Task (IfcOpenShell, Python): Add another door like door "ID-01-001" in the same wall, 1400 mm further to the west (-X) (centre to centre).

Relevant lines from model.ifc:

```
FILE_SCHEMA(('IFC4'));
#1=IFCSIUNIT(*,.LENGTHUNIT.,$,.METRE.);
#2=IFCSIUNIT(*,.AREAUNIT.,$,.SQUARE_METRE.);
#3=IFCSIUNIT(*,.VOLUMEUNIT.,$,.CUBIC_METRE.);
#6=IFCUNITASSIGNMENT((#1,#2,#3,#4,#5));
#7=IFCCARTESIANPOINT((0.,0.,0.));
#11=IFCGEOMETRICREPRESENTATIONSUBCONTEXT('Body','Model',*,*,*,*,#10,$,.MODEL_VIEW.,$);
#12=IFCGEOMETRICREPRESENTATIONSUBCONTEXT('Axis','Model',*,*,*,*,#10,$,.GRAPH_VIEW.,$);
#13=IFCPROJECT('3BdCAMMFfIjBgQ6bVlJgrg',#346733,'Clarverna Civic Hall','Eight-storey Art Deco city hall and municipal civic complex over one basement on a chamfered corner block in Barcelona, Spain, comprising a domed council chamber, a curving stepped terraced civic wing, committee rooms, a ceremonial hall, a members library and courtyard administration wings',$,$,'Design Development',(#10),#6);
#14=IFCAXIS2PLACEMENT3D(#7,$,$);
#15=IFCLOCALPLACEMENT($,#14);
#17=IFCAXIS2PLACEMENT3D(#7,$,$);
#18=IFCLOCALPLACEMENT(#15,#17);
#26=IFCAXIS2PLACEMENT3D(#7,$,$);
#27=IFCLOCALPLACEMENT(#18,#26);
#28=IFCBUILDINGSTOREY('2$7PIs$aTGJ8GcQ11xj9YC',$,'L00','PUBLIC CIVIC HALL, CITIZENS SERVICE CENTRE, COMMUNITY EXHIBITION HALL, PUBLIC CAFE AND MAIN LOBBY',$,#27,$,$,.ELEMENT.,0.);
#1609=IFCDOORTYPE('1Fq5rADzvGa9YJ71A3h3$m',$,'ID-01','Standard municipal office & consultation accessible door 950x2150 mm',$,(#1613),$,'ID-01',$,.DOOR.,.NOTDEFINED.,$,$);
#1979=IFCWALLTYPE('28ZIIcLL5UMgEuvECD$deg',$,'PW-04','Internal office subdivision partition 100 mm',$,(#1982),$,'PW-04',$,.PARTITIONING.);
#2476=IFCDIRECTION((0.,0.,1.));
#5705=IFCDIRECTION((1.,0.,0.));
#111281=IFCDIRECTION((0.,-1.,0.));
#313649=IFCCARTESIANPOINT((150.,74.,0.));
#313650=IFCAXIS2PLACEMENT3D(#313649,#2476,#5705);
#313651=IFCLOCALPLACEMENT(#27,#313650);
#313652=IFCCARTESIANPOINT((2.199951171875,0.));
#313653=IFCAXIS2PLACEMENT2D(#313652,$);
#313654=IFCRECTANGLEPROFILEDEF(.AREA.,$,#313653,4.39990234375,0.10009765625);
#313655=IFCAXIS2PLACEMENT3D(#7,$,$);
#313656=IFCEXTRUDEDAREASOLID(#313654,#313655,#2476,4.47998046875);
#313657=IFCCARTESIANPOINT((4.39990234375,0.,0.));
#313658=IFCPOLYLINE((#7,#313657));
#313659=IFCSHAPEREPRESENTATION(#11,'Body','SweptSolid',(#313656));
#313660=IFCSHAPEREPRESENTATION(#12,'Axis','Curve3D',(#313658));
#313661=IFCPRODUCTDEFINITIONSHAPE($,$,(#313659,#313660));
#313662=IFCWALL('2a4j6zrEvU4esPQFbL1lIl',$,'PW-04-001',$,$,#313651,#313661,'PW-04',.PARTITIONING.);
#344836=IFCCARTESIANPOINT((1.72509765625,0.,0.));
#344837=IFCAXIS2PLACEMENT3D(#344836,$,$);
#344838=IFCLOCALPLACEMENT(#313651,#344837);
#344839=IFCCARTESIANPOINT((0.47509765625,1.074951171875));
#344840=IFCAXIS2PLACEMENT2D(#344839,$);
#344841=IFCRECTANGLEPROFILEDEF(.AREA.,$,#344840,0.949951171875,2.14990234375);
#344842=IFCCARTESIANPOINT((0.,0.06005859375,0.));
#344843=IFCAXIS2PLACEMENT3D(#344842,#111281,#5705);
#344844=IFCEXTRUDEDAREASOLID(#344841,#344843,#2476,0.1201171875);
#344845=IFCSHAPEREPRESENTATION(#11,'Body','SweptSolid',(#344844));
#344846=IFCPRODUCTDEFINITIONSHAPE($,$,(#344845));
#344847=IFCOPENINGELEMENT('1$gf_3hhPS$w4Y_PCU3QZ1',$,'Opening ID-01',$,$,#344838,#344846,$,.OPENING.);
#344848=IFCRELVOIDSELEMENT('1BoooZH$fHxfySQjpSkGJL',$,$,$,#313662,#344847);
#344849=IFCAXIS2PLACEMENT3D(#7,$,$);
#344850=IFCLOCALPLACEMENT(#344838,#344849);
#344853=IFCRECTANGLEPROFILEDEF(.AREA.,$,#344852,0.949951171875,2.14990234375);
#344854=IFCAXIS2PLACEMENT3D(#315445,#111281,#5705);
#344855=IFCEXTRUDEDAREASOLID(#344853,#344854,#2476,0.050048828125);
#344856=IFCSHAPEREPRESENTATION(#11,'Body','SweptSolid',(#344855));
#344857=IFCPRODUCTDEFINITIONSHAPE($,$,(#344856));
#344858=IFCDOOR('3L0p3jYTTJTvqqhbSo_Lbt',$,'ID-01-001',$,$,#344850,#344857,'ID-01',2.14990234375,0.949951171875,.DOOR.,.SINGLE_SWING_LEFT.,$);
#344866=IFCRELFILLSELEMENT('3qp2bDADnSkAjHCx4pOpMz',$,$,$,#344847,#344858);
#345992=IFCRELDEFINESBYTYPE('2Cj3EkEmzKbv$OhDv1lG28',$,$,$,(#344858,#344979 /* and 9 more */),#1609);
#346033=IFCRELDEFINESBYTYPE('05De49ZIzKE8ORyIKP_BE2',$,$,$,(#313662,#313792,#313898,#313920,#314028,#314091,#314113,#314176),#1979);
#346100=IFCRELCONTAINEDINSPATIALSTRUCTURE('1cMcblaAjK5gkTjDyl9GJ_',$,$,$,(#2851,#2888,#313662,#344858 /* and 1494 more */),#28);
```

```python
import ifcopenshell
import ifcopenshell.api.feature
import ifcopenshell.api.geometry
import ifcopenshell.api.root
import ifcopenshell.geom
import ifcopenshell.util.element
import ifcopenshell.util.placement
import ifcopenshell.util.shape
import ifcopenshell.util.unit

model = ifcopenshell.open("model.ifc")
unit_scale = ifcopenshell.util.unit.calculate_unit_scale(model)
settings = ifcopenshell.geom.settings()


def volume(element):
    """Net volume in cubic metres, openings subtracted."""
    shape = ifcopenshell.geom.create_shape(settings, element)
    return ifcopenshell.util.shape.get_volume(shape.geometry)


door = model.by_id(344858)
opening = door.FillsVoids[0].RelatingOpeningElement
wall = opening.VoidsElements[0].RelatingBuildingElement
before = volume(wall)
shift = ifcopenshell.util.placement.get_local_placement(wall.ObjectPlacement)[:3, 0] * -1.4 / unit_scale

# copy_class copies the void relationship, type, container and properties, but no geometry.
new_opening = ifcopenshell.api.root.copy_class(model, product=opening)
new_opening.Representation = ifcopenshell.util.element.copy_deep(
    model, opening.Representation, exclude=["IfcGeometricRepresentationContext", "IfcRepresentationMap"]
)
new_door = ifcopenshell.api.root.copy_class(model, product=door)
new_door.Representation = ifcopenshell.util.element.copy_deep(
    model, door.Representation, exclude=["IfcGeometricRepresentationContext", "IfcRepresentationMap"]
)
new_door.Tag = None
ifcopenshell.api.feature.add_filling(model, opening=new_opening, element=new_door)

for old, new in ((opening, new_opening), (door, new_door)):
    matrix = ifcopenshell.util.placement.get_local_placement(old.ObjectPlacement)
    matrix[:3, 3] += shift
    ifcopenshell.api.geometry.edit_object_placement(model, product=new, matrix=matrix, is_si=False)

after = volume(wall)

print(f"wall volume {before:.3f} -> {after:.3f} m3")

model.write("model-out.ifc")
```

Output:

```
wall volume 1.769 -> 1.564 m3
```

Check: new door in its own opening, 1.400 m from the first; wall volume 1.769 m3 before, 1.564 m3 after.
